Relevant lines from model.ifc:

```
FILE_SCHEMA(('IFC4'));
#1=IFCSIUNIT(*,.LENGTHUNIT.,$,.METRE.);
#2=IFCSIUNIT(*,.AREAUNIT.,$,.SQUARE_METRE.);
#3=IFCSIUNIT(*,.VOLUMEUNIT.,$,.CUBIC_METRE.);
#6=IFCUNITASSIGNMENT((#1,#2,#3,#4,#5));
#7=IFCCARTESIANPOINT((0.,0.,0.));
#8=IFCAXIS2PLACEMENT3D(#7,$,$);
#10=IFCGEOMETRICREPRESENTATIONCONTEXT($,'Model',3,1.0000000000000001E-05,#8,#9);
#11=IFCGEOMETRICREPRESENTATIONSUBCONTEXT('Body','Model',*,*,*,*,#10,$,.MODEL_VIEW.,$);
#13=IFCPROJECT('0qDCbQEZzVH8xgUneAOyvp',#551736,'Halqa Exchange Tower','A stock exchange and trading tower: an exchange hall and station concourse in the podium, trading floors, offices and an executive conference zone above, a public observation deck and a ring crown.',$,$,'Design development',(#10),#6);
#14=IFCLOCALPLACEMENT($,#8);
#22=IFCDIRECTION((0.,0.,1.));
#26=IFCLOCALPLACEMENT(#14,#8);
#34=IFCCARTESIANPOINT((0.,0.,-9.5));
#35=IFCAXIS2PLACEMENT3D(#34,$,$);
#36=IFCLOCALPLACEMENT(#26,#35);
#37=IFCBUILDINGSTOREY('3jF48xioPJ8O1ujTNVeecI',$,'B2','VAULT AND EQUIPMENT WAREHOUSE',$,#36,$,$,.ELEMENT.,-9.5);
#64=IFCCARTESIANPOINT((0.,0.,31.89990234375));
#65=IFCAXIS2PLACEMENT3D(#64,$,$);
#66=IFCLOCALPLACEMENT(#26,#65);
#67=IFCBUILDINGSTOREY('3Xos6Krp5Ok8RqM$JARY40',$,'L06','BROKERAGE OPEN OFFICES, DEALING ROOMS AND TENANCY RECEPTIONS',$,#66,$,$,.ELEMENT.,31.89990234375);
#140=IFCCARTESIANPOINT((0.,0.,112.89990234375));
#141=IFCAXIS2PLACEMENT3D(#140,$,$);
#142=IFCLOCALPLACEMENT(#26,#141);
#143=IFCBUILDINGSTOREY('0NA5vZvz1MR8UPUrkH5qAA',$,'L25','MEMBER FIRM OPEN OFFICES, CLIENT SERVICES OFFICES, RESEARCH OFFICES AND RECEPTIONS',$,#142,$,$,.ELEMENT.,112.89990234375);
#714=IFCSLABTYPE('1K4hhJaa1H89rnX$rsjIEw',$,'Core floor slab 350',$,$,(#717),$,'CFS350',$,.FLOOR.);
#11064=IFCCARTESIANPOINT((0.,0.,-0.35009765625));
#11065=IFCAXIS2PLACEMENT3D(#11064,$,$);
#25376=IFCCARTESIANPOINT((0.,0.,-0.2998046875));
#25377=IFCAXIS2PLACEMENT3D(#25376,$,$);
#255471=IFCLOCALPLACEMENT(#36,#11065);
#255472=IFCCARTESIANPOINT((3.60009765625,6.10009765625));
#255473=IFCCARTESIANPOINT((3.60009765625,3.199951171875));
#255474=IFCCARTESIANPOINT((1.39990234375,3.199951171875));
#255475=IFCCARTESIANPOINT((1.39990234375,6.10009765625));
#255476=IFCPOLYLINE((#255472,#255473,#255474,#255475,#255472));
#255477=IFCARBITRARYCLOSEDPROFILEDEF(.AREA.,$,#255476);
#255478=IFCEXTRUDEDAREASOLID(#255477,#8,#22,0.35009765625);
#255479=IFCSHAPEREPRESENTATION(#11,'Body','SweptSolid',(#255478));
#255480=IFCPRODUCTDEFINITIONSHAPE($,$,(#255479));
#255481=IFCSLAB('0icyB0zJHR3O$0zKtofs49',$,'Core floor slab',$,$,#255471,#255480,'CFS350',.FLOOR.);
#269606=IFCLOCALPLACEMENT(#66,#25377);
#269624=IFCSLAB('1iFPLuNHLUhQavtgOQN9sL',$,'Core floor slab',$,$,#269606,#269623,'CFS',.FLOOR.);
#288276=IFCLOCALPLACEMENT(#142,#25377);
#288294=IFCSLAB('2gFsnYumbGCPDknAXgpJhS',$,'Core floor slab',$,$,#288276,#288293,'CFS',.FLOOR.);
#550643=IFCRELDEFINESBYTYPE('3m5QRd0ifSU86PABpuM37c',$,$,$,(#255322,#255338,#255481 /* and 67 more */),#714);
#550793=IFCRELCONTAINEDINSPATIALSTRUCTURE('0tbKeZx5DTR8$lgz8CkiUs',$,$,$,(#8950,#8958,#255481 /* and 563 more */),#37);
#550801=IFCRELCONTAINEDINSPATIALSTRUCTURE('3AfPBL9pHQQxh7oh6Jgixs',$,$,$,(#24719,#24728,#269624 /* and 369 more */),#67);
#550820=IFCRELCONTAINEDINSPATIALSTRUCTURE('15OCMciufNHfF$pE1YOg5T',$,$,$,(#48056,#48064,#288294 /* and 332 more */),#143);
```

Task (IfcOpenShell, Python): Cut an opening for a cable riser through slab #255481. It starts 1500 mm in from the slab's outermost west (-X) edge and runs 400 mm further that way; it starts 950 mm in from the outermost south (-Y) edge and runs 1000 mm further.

```python
import numpy as np
import ifcopenshell
import ifcopenshell.api.feature
import ifcopenshell.api.geometry
import ifcopenshell.api.root
import ifcopenshell.geom
import ifcopenshell.util.placement
import ifcopenshell.util.representation
import ifcopenshell.util.shape
import ifcopenshell.util.unit

model = ifcopenshell.open("model.ifc")
unit_scale = ifcopenshell.util.unit.calculate_unit_scale(model)
settings = ifcopenshell.geom.settings()


def volume(element):
    """Net volume in cubic metres, openings subtracted."""
    shape = ifcopenshell.geom.create_shape(settings, element)
    return ifcopenshell.util.shape.get_volume(shape.geometry)


slab = model.by_guid("0icyB0zJHR3O$0zKtofs49")
before = volume(slab)

# Extent in the slab's own axes, in metres. The edges named are its -X and -Y sides.
slab_shape = ifcopenshell.geom.create_shape(settings, slab)
vertices = ifcopenshell.util.shape.get_vertices(slab_shape.geometry)
x_min, y_min, bottom = vertices.min(axis=0)
top = vertices[:, 2].max()

opening = ifcopenshell.api.root.create_entity(model, ifc_class="IfcOpeningElement", name="Cable riser opening", predefined_type="OPENING")
context = ifcopenshell.util.representation.get_context(model, "Model", "Body", "MODEL_VIEW")
width, depth = 0.4, 1
outline = [(0.0, 0.0), (width, 0.0), (width, depth), (0.0, depth), (0.0, 0.0)]
# Overshoot both faces by 50 mm so the cut is clean.
shape = ifcopenshell.api.geometry.add_slab_representation(
    model, context=context, depth=top - bottom + 0.1, polyline=outline
)
ifcopenshell.api.geometry.assign_representation(model, product=opening, representation=shape)

matrix = ifcopenshell.util.placement.get_local_placement(slab.ObjectPlacement)
matrix[:, 3] = matrix @ np.append(np.array([x_min + 1.5, y_min + 0.95, bottom - 0.05]) / unit_scale, 1.0)
ifcopenshell.api.geometry.edit_object_placement(model, product=opening, matrix=matrix, is_si=False)
ifcopenshell.api.feature.add_feature(model, feature=opening, element=slab)

after = volume(slab)

print(f"slab volume {before:.3f} -> {after:.3f} m3")

model.write("model_v2.ifc")
```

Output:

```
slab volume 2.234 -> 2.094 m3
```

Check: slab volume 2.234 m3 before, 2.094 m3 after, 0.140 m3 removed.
